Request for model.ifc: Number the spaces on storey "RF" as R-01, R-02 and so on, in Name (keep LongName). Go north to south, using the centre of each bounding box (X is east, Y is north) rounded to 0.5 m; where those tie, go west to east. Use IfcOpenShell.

First a look at what the model holds.

```python
import ifcopenshell
import ifcopenshell.util.element
import ifcopenshell.util.placement

model = ifcopenshell.open("model.ifc")
print(model.schema)
storey = next(s for s in model.by_type("IfcBuildingStorey") if s.Name == "RF")
spaces = [e for e in ifcopenshell.util.element.get_decomposition(storey) if e.is_a("IfcSpace")]
for e in sorted(spaces, key=lambda e: e.id()):
    origin = ifcopenshell.util.placement.get_local_placement(e.ObjectPlacement)[:3, 3]
    print(e.id(), e.Name, e.LongName, origin.round(2) + 0.0, sep=" | ")
```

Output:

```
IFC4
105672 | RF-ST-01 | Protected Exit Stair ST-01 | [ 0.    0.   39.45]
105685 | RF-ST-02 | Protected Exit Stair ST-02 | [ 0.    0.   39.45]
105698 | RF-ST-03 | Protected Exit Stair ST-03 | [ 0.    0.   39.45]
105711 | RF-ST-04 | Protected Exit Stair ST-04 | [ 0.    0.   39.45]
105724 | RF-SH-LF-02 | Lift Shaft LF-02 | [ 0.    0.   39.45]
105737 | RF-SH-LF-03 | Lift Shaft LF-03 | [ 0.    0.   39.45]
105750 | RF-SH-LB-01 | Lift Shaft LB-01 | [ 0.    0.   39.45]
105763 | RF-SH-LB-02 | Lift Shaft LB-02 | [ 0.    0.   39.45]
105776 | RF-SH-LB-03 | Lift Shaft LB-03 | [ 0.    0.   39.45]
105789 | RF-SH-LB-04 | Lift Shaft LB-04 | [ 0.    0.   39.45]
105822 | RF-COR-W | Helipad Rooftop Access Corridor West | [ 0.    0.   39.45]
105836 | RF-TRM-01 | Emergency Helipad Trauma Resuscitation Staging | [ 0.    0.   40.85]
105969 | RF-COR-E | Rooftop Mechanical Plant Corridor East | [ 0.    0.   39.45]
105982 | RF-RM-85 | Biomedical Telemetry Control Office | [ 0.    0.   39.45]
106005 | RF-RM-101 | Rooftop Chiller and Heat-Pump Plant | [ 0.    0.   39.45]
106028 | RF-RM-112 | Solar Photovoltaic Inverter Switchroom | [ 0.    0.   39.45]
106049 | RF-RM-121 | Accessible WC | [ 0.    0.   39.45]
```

```python
import ifcopenshell
import ifcopenshell.geom
import ifcopenshell.util.element
import ifcopenshell.util.shape

model = ifcopenshell.open("model.ifc")
settings = ifcopenshell.geom.settings()
settings.set("use-world-coords", True)


def centre(element):
    shape = ifcopenshell.geom.create_shape(settings, element)
    return ifcopenshell.util.shape.get_bbox_centroid(shape.geometry)


storey = next(s for s in model.by_type("IfcBuildingStorey") if s.Name == "RF")
spaces = [e for e in ifcopenshell.util.element.get_decomposition(storey) if e.is_a("IfcSpace")]

# Insertion points can sit at a corner or the storey origin, so sort by the geometry (in metres).
centres = {e: centre(e) for e in spaces}
spaces.sort(key=lambda e: (-round(centres[e][1] / 0.5), centres[e][0]))

for i, e in enumerate(spaces, start=1):
    number = f"R-{i:02d}"
    e.Name = number
    print(e.id(), number)

model.write("model_updated.ifc")
```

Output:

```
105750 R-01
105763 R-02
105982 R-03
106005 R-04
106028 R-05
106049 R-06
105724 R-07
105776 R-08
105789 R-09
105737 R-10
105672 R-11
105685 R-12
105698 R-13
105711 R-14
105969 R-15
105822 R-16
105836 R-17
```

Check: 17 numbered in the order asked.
